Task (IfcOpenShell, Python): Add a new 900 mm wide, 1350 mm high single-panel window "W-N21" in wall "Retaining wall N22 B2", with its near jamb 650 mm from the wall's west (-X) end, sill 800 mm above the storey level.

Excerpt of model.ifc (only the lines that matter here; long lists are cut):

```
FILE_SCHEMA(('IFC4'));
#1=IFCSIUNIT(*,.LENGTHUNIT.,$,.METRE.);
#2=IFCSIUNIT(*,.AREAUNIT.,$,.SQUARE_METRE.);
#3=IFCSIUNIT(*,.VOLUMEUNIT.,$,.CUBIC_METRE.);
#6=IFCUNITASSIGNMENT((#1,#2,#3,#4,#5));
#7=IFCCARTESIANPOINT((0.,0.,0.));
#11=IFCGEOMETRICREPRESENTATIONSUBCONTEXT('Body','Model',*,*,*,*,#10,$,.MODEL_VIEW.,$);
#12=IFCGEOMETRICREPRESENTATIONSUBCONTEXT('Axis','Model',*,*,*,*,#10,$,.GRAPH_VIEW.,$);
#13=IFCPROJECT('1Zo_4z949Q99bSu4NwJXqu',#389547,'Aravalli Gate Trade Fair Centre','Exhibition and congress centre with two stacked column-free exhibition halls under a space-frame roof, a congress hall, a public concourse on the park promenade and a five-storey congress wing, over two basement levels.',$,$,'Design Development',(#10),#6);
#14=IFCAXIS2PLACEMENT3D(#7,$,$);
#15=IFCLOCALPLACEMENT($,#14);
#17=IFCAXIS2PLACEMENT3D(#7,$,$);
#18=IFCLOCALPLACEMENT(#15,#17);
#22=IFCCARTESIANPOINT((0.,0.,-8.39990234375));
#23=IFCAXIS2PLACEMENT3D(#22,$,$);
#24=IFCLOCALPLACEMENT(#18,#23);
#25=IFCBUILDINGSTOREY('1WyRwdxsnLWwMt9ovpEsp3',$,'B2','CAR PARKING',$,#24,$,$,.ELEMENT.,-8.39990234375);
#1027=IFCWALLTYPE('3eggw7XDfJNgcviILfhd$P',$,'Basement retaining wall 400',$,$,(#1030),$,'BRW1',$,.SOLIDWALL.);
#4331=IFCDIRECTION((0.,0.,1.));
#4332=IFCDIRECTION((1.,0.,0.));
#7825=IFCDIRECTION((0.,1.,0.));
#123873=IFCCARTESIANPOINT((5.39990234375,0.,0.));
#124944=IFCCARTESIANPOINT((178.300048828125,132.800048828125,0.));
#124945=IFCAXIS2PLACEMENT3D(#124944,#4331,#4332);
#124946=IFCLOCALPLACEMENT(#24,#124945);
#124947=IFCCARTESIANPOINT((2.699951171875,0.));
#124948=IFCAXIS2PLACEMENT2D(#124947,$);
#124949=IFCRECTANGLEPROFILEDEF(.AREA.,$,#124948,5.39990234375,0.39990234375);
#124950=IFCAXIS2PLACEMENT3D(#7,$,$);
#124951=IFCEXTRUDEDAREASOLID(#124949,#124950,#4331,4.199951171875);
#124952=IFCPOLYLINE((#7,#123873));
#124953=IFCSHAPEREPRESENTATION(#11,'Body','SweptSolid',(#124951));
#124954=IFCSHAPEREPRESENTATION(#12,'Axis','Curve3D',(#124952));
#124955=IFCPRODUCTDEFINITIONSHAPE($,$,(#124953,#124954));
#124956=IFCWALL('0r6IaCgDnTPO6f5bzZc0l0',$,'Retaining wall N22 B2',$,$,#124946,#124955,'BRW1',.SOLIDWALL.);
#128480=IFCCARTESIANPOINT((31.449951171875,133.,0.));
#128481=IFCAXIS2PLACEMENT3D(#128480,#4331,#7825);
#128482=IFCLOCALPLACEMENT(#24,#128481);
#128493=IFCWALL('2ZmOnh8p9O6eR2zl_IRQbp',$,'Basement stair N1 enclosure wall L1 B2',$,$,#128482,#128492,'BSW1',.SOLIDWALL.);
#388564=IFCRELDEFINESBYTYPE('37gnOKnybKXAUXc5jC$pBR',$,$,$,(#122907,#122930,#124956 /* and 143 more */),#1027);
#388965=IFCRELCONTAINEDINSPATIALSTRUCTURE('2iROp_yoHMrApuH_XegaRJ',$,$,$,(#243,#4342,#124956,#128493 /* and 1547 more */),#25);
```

```python
import numpy as np
import ifcopenshell
import ifcopenshell.api.feature
import ifcopenshell.api.geometry
import ifcopenshell.api.root
import ifcopenshell.api.spatial
import ifcopenshell.geom
import ifcopenshell.util.element
import ifcopenshell.util.placement
import ifcopenshell.util.representation
import ifcopenshell.util.shape
import ifcopenshell.util.unit

model = ifcopenshell.open("model.ifc")
unit_scale = ifcopenshell.util.unit.calculate_unit_scale(model)
settings = ifcopenshell.geom.settings()


def volume(element):
    """Net volume in cubic metres, openings subtracted."""
    shape = ifcopenshell.geom.create_shape(settings, element)
    return ifcopenshell.util.shape.get_volume(shape.geometry)


wall = model.by_id(124956)
storey = ifcopenshell.util.element.get_container(wall, ifc_class="IfcBuildingStorey")
context = ifcopenshell.util.representation.get_context(model, "Model", "Body", "MODEL_VIEW")
before = volume(wall)

width, height, from_end, sill = 0.9, 1.35, 0.65, 0.8  # metres

# The wall runs along its own X axis, and the end named is its -X end.
wall_shape = ifcopenshell.geom.create_shape(settings, wall)
x, y, z = ifcopenshell.util.shape.get_vertices(wall_shape.geometry).T
start = x.min() + from_end
face, thickness = float(y.min()), float(y.max() - y.min())
wall_matrix = ifcopenshell.util.placement.get_local_placement(wall.ObjectPlacement)
level = ifcopenshell.util.placement.get_local_placement(storey.ObjectPlacement)[2, 3]


def in_wall(x, y):
    """Placement at x, y metres in the wall's axes, at sill height."""
    matrix = wall_matrix.copy()
    matrix[:, 3] = wall_matrix @ np.array([x / unit_scale, y / unit_scale, 0.0, 1.0])
    matrix[2, 3] = level + sill / unit_scale
    return matrix


# Opening: a box that overshoots both wall faces by 50 mm.
opening = ifcopenshell.api.root.create_entity(model, ifc_class="IfcOpeningElement", predefined_type="OPENING")
box = ifcopenshell.api.geometry.add_wall_representation(
    model, context=context, length=width, height=height, thickness=thickness + 0.1
)
ifcopenshell.api.geometry.assign_representation(model, product=opening, representation=box)
ifcopenshell.api.geometry.edit_object_placement(model, product=opening, matrix=in_wall(start, face - 0.05), is_si=False)
ifcopenshell.api.feature.add_feature(model, feature=opening, element=wall)

window = ifcopenshell.api.root.create_entity(model, ifc_class="IfcWindow", name="W-N21", predefined_type="WINDOW")
window.OverallWidth, window.OverallHeight = width / unit_scale, height / unit_scale
window.PartitioningType = "SINGLE_PANEL"
body = ifcopenshell.api.geometry.add_window_representation(
    model,
    context=context,
    overall_width=window.OverallWidth,
    overall_height=window.OverallHeight,
    partition_type="SINGLE_PANEL",
)
ifcopenshell.api.geometry.assign_representation(model, product=window, representation=body)
ifcopenshell.api.spatial.assign_container(model, products=[window], relating_structure=storey)
ifcopenshell.api.feature.add_filling(model, opening=opening, element=window)

# Centre the window in the wall's thickness.
ifcopenshell.api.geometry.edit_object_placement(model, product=window, matrix=in_wall(start, face), is_si=False)
window_shape = ifcopenshell.geom.create_shape(settings, window)
depth = ifcopenshell.util.shape.get_vertices(window_shape.geometry)[:, 1]
offset = face + thickness / 2 - (depth.min() + depth.max()) / 2
ifcopenshell.api.geometry.edit_object_placement(model, product=window, matrix=in_wall(start, offset), is_si=False)

after = volume(wall)

print(f"wall volume {before:.3f} -> {after:.3f} m3")

model.write("model-out.ifc")
```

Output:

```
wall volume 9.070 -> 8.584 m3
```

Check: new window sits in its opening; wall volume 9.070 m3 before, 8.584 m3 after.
